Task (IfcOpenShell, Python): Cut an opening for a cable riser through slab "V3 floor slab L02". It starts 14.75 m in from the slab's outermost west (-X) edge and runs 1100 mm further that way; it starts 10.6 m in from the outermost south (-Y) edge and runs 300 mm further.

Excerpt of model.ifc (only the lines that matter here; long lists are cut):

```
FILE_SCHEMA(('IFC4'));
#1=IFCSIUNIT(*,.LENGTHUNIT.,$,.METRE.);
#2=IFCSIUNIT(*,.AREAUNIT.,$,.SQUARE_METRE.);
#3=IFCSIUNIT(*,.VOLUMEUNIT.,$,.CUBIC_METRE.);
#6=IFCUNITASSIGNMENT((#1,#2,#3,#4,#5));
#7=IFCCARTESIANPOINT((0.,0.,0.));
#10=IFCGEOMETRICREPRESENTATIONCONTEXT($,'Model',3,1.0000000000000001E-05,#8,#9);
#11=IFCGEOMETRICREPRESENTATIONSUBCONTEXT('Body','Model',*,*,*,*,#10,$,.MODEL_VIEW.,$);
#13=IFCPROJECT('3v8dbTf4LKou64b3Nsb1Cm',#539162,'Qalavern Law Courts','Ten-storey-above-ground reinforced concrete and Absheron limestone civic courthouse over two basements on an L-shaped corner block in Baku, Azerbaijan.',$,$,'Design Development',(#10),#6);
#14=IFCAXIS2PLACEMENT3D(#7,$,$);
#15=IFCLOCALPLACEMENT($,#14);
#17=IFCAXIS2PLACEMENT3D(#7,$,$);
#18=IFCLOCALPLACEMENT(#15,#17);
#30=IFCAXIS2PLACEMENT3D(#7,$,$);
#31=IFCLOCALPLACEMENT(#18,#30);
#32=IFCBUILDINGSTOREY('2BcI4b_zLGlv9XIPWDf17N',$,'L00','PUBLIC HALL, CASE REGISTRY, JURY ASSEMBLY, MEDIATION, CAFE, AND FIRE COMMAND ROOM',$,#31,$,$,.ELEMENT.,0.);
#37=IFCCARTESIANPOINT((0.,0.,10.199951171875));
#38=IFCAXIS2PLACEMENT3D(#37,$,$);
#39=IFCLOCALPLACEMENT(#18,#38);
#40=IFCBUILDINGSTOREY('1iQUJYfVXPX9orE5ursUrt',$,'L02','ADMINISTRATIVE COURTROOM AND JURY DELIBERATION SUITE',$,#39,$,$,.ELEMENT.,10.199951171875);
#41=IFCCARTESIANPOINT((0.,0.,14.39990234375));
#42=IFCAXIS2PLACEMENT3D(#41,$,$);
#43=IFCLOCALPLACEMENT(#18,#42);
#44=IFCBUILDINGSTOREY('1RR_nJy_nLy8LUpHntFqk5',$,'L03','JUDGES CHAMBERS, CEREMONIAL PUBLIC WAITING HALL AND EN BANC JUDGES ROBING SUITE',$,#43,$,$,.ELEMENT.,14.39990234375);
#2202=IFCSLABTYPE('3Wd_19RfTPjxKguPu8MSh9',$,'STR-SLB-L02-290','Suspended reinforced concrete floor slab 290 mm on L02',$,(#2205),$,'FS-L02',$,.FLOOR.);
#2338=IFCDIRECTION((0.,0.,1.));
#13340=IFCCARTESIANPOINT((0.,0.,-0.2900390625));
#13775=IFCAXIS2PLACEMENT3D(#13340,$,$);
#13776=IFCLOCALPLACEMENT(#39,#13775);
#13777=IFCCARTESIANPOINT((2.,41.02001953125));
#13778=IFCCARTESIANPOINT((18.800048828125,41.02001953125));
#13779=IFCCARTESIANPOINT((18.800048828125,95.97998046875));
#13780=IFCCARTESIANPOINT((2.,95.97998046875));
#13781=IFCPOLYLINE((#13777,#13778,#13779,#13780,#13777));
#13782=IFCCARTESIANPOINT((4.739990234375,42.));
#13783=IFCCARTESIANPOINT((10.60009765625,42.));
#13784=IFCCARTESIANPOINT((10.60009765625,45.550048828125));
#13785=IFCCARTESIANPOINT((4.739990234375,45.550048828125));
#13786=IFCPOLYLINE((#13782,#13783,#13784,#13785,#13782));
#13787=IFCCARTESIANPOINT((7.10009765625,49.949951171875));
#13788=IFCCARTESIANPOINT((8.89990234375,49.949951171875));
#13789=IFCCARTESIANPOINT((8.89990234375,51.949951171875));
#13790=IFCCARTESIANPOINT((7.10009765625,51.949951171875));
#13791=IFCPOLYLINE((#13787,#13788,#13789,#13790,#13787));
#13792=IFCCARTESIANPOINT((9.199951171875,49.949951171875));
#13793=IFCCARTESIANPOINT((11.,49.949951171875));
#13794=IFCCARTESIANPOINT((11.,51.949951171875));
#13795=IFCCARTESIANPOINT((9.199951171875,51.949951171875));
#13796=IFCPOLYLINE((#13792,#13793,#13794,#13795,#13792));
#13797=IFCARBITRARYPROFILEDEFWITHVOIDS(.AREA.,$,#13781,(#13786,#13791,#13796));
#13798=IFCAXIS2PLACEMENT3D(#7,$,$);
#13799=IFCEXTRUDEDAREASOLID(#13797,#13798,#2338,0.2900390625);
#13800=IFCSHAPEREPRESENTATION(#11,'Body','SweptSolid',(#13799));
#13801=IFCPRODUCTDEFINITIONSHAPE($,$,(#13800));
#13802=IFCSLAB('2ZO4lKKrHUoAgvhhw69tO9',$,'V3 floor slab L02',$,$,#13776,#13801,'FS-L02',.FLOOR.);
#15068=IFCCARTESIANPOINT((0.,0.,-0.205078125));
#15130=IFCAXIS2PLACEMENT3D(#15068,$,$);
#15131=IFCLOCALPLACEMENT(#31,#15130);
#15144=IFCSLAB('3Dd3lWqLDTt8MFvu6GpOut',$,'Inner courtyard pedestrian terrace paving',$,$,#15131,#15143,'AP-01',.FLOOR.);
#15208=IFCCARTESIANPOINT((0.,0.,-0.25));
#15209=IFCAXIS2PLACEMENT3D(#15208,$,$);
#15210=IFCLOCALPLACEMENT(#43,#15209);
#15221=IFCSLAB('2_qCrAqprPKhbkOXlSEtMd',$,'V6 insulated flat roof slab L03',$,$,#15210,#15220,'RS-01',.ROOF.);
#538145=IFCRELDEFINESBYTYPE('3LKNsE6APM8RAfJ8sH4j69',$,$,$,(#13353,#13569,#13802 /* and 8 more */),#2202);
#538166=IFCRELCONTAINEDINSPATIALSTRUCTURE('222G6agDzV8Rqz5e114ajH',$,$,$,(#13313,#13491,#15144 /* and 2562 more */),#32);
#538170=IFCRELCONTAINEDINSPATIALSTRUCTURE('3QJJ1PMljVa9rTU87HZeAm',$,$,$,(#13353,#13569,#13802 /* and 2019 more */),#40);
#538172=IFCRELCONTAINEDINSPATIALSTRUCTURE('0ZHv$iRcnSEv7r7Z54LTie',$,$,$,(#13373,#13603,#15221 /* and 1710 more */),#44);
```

```python
import numpy as np
import ifcopenshell
import ifcopenshell.api.feature
import ifcopenshell.api.geometry
import ifcopenshell.api.root
import ifcopenshell.geom
import ifcopenshell.util.placement
import ifcopenshell.util.representation
import ifcopenshell.util.shape
import ifcopenshell.util.unit

model = ifcopenshell.open("model.ifc")
unit_scale = ifcopenshell.util.unit.calculate_unit_scale(model)
settings = ifcopenshell.geom.settings()


def volume(element):
    """Net volume in cubic metres, openings subtracted."""
    shape = ifcopenshell.geom.create_shape(settings, element)
    return ifcopenshell.util.shape.get_volume(shape.geometry)


slab = model.by_guid("2ZO4lKKrHUoAgvhhw69tO9")
before = volume(slab)

# Extent in the slab's own axes, in metres. The edges named are its -X and -Y sides.
slab_shape = ifcopenshell.geom.create_shape(settings, slab)
vertices = ifcopenshell.util.shape.get_vertices(slab_shape.geometry)
x_min, y_min, bottom = vertices.min(axis=0)
top = vertices[:, 2].max()

opening = ifcopenshell.api.root.create_entity(model, ifc_class="IfcOpeningElement", name="Cable riser opening", predefined_type="OPENING")
context = ifcopenshell.util.representation.get_context(model, "Model", "Body", "MODEL_VIEW")
width, depth = 1.1, 0.3
outline = [(0.0, 0.0), (width, 0.0), (width, depth), (0.0, depth), (0.0, 0.0)]
# Overshoot both faces by 50 mm so the cut is clean.
shape = ifcopenshell.api.geometry.add_slab_representation(
    model, context=context, depth=top - bottom + 0.1, polyline=outline
)
ifcopenshell.api.geometry.assign_representation(model, product=opening, representation=shape)

matrix = ifcopenshell.util.placement.get_local_placement(slab.ObjectPlacement)
matrix[:, 3] = matrix @ np.append(np.array([x_min + 14.75, y_min + 10.6, bottom - 0.05]) / unit_scale, 1.0)
ifcopenshell.api.geometry.edit_object_placement(model, product=opening, matrix=matrix, is_si=False)
ifcopenshell.api.feature.add_feature(model, feature=opening, element=slab)

after = volume(slab)

print(f"slab volume {before:.3f} -> {after:.3f} m3")

model.write("model_edited.ifc")
```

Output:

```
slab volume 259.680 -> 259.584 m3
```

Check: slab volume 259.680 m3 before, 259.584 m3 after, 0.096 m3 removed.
